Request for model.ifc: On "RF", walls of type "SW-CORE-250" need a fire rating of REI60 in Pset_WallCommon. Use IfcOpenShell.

First a look at what the model holds.

```python
import ifcopenshell
import ifcopenshell.util.element

model = ifcopenshell.open("model.ifc")
print(model.schema)
storey = next(s for s in model.by_type("IfcBuildingStorey") if s.Name == "RF")
walls = [e for e in ifcopenshell.util.element.get_decomposition(storey) if e.is_a("IfcWall")]
seen = {}
for e in walls:
    element_type = ifcopenshell.util.element.get_type(e)
    key = (element_type.Name if element_type != e and element_type else None, ifcopenshell.util.element.get_pset(e, "Pset_WallCommon", "FireRating"))
    seen[key] = seen.get(key, 0) + 1
for (name, value), count in sorted(seen.items(), key=str):
    print(count, "x", name, "|", value)
```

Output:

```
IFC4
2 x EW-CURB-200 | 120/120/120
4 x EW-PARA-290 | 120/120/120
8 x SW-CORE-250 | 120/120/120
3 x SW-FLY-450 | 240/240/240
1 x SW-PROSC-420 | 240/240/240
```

```python
import ifcopenshell
import ifcopenshell.api.pset
import ifcopenshell.util.element

model = ifcopenshell.open("model.ifc")

storey = next(s for s in model.by_type("IfcBuildingStorey") if s.Name == "RF")
walls = [e for e in ifcopenshell.util.element.get_decomposition(storey) if e.is_a("IfcWall")]

count = 0
for e in walls:
    element_type = ifcopenshell.util.element.get_type(e)
    if element_type in (None, e) or element_type.Name != "SW-CORE-250":
        continue
    # add_pset returns the element's existing set when there is one.
    pset = ifcopenshell.api.pset.add_pset(model, product=e, name="Pset_WallCommon")
    ifcopenshell.api.pset.edit_pset(model, pset=pset, properties={"FireRating": "REI60"})
    count += 1

print(count, "walls updated")

model.write("model_v2.ifc")
```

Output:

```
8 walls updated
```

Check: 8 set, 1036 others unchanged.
